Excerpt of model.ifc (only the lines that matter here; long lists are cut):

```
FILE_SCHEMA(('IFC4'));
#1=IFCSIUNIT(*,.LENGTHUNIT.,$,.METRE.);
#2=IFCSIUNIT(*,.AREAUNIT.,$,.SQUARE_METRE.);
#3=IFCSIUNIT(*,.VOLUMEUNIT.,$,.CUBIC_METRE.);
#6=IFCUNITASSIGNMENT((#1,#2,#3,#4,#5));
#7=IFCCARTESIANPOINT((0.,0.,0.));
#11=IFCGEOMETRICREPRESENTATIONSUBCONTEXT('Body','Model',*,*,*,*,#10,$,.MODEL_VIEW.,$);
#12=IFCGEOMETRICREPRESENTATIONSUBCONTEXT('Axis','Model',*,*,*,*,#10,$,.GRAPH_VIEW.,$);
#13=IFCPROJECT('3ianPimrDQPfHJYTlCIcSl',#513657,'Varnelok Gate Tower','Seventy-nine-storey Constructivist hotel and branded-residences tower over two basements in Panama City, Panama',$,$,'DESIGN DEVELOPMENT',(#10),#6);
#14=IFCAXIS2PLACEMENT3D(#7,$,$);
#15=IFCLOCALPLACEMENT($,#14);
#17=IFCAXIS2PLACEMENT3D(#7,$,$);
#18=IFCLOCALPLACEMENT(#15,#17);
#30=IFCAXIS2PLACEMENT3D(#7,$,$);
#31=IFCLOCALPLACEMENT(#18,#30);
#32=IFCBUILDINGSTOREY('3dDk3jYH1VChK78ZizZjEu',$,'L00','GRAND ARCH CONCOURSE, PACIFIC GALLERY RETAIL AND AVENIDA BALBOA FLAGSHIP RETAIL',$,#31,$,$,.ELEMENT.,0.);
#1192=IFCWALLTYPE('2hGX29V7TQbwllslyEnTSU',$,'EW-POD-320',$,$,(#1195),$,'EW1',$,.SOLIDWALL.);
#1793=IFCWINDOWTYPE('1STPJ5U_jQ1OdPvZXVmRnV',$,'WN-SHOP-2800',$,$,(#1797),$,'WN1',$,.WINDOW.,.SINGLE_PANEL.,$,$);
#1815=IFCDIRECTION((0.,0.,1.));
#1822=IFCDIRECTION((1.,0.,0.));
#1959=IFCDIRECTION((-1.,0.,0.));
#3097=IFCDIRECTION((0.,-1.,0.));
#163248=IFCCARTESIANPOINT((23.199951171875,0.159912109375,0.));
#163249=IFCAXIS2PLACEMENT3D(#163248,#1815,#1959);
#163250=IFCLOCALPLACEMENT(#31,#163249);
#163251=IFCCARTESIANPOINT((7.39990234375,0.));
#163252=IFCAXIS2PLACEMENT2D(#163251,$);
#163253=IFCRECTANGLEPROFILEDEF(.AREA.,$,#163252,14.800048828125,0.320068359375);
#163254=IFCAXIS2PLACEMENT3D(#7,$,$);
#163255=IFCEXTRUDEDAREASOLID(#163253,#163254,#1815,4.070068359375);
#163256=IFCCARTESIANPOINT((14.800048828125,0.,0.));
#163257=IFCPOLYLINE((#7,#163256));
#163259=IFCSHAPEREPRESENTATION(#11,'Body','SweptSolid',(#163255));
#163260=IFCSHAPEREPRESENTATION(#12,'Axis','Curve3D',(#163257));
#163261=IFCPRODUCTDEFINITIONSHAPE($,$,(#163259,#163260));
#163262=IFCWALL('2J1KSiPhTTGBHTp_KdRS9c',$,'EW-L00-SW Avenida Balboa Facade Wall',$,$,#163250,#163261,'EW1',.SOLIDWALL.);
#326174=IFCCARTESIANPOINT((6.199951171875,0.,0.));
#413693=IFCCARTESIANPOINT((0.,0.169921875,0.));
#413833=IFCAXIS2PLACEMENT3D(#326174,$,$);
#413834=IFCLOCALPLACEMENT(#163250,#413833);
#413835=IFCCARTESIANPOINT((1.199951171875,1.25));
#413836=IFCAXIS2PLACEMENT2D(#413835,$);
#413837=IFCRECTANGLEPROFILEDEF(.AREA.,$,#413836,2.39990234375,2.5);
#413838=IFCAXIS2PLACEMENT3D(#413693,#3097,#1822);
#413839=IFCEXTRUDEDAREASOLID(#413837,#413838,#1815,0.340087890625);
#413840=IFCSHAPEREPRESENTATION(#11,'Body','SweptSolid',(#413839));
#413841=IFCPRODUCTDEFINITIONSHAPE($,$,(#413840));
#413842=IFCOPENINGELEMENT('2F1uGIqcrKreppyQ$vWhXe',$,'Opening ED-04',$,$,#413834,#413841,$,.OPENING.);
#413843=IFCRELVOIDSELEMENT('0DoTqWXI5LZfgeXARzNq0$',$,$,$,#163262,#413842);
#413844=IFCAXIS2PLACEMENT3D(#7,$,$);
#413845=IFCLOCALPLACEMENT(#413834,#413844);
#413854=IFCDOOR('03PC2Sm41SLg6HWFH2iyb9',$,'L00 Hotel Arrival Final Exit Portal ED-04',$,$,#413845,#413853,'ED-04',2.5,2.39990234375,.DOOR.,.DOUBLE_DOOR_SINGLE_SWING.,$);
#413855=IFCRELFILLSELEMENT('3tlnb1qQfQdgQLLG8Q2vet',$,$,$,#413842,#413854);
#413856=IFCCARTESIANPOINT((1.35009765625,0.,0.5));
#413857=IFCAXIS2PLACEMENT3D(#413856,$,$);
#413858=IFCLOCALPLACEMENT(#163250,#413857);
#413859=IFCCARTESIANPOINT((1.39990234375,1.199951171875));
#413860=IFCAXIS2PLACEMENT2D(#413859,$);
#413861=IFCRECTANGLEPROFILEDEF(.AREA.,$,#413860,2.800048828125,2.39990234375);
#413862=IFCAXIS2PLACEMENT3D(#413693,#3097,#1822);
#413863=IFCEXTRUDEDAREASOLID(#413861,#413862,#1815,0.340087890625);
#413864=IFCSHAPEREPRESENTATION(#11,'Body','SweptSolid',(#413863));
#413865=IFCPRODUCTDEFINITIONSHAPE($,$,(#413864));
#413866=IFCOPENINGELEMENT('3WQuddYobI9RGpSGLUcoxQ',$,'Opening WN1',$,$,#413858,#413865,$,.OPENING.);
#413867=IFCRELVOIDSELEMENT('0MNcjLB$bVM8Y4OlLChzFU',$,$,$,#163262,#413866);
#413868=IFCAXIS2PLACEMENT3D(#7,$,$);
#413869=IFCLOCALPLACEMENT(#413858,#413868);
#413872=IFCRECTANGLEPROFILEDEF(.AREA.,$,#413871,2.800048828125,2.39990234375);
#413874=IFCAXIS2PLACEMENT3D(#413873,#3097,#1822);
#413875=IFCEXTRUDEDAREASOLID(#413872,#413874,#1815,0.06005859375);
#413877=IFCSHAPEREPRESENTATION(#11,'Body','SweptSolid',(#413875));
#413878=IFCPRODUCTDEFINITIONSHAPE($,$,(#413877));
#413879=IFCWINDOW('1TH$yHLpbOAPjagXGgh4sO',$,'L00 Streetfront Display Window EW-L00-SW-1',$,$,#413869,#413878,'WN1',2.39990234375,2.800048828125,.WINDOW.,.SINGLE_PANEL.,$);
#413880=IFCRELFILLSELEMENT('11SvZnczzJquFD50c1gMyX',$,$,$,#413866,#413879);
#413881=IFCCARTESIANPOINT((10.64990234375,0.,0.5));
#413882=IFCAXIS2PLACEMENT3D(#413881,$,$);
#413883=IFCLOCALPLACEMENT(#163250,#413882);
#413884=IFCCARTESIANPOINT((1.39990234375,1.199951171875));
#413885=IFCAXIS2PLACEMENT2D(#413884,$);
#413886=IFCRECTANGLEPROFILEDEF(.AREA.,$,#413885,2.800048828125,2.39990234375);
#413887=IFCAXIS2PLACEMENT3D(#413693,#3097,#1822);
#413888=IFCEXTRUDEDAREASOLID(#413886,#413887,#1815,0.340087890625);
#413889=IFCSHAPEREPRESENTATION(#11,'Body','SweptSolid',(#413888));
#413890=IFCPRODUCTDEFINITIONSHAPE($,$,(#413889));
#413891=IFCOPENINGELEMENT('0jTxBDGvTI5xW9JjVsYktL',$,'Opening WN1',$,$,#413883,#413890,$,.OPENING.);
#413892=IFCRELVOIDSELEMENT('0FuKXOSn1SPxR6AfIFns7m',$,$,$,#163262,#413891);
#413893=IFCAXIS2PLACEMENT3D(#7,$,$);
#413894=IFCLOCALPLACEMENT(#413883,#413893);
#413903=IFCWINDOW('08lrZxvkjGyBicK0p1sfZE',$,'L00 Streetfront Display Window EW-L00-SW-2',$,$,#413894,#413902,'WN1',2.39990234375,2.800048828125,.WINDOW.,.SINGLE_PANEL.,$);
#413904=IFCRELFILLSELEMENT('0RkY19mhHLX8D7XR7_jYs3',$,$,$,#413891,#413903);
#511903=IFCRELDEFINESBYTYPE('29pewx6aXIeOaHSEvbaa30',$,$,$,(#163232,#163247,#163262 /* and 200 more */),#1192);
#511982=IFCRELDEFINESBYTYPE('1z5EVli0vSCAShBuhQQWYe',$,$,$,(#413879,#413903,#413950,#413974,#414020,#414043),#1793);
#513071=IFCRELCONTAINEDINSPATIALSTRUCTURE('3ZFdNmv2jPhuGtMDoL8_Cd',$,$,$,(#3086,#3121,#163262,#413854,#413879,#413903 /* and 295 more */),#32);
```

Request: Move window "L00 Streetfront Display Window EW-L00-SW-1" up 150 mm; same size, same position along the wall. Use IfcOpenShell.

```python
import numpy as np
import ifcopenshell
import ifcopenshell.api.geometry
import ifcopenshell.util.placement
import ifcopenshell.util.unit

model = ifcopenshell.open("model.ifc")
unit_scale = ifcopenshell.util.unit.calculate_unit_scale(model)

window = model.by_guid("1TH$yHLpbOAPjagXGgh4sO")
opening = window.FillsVoids[0].RelatingOpeningElement
dz = 0.15

shift = np.array([0.0, 0.0, dz])
# The window is placed relative to its opening, so it follows when the opening moves.
matrix = ifcopenshell.util.placement.get_local_placement(opening.ObjectPlacement)
matrix[:3, 3] += shift
ifcopenshell.api.geometry.edit_object_placement(
    model, product=opening, matrix=matrix, is_si=False, should_transform_children=True
)

print(f"moved by {dz * unit_scale:+.3f} m")

model.write("model_updated.ifc")
```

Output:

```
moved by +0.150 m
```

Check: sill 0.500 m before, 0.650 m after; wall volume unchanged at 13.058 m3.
